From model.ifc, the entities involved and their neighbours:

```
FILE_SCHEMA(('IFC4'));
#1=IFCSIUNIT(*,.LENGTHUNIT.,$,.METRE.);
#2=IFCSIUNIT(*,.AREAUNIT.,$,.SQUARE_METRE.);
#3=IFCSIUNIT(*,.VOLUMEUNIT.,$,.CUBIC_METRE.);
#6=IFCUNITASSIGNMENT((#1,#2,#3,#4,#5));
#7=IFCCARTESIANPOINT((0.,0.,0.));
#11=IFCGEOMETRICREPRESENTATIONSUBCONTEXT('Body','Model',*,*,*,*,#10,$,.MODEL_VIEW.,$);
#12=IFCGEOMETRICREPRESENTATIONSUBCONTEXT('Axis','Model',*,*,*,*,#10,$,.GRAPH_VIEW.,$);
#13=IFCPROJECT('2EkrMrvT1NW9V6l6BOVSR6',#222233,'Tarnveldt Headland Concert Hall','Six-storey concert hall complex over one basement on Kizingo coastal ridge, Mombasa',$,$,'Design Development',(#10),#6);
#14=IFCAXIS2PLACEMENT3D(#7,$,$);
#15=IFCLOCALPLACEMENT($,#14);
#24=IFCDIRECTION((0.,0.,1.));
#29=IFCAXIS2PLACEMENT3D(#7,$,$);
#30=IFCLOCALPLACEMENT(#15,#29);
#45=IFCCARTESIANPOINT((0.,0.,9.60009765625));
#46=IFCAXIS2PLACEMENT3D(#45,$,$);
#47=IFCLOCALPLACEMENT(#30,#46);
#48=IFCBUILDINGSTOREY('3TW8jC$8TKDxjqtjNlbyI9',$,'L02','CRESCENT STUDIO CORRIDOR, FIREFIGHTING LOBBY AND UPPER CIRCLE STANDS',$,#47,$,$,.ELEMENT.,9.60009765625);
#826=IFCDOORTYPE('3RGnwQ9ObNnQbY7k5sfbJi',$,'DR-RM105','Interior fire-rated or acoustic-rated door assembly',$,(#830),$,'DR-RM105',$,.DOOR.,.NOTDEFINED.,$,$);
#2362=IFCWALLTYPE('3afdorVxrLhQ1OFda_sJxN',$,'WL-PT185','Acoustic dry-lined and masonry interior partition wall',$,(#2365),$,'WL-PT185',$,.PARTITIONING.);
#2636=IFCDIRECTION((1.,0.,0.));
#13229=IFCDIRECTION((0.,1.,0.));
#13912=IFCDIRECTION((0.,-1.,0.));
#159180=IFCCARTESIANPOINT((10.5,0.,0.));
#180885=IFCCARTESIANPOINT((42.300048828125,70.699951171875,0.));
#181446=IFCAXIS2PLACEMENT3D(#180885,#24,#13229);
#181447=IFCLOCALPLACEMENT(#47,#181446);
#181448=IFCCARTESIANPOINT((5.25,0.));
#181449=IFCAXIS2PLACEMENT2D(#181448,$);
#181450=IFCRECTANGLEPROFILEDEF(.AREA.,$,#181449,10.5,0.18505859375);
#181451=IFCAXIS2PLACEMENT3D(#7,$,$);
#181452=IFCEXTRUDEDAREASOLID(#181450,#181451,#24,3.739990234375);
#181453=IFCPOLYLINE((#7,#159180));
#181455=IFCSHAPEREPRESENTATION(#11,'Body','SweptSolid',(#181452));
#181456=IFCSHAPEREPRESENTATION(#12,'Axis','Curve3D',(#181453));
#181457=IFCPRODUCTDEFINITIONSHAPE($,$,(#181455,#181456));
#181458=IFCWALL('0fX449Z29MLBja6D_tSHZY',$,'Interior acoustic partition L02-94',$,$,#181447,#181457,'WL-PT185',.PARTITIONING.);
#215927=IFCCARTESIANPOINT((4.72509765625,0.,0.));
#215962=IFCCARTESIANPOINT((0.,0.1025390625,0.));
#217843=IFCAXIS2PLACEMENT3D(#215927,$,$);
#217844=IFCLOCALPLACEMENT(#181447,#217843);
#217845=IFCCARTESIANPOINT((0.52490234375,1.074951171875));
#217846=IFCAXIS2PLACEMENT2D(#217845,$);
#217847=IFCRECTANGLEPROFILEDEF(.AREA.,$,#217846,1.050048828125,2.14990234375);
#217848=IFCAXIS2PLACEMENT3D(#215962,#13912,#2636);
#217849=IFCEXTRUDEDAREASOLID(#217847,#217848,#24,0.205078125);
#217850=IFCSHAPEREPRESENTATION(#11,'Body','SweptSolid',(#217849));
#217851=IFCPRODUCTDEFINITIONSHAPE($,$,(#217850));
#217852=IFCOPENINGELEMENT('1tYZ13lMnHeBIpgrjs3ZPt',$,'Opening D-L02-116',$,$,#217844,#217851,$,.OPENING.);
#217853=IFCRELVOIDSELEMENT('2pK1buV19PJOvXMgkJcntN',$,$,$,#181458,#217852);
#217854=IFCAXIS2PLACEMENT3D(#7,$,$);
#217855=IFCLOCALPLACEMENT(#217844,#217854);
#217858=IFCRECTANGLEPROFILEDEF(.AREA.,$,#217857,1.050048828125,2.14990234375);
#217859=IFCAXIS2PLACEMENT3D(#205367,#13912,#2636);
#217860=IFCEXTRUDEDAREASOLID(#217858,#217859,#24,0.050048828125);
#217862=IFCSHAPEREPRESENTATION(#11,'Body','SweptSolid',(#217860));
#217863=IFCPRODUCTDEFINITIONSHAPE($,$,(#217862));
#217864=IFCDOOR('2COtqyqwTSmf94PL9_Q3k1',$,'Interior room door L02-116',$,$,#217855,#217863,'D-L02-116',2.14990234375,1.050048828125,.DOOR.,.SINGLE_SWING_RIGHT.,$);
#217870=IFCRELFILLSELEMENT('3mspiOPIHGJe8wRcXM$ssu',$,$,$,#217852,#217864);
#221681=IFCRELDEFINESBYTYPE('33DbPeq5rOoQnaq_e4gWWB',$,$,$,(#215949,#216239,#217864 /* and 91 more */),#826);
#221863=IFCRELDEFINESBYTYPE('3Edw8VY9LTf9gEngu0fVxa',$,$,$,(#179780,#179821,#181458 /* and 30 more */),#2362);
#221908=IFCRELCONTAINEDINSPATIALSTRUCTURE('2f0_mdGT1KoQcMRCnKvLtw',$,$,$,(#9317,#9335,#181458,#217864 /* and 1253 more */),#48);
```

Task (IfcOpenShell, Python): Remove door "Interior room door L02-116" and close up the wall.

```python
import ifcopenshell
import ifcopenshell.api.feature
import ifcopenshell.api.root
import ifcopenshell.geom
import ifcopenshell.util.shape

model = ifcopenshell.open("model.ifc")
settings = ifcopenshell.geom.settings()


def volume(element):
    """Net volume in cubic metres, openings subtracted."""
    shape = ifcopenshell.geom.create_shape(settings, element)
    return ifcopenshell.util.shape.get_volume(shape.geometry)


door = model.by_guid("2COtqyqwTSmf94PL9_Q3k1")
opening = door.FillsVoids[0].RelatingOpeningElement
wall = opening.VoidsElements[0].RelatingBuildingElement
before = volume(wall)

ifcopenshell.api.root.remove_product(model, product=door)
ifcopenshell.api.feature.remove_feature(model, feature=opening)

after = volume(wall)

print(f"wall volume {before:.3f} -> {after:.3f} m3")

model.write("model_v2.ifc")
```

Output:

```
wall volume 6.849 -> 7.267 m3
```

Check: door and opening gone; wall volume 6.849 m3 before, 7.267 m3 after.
